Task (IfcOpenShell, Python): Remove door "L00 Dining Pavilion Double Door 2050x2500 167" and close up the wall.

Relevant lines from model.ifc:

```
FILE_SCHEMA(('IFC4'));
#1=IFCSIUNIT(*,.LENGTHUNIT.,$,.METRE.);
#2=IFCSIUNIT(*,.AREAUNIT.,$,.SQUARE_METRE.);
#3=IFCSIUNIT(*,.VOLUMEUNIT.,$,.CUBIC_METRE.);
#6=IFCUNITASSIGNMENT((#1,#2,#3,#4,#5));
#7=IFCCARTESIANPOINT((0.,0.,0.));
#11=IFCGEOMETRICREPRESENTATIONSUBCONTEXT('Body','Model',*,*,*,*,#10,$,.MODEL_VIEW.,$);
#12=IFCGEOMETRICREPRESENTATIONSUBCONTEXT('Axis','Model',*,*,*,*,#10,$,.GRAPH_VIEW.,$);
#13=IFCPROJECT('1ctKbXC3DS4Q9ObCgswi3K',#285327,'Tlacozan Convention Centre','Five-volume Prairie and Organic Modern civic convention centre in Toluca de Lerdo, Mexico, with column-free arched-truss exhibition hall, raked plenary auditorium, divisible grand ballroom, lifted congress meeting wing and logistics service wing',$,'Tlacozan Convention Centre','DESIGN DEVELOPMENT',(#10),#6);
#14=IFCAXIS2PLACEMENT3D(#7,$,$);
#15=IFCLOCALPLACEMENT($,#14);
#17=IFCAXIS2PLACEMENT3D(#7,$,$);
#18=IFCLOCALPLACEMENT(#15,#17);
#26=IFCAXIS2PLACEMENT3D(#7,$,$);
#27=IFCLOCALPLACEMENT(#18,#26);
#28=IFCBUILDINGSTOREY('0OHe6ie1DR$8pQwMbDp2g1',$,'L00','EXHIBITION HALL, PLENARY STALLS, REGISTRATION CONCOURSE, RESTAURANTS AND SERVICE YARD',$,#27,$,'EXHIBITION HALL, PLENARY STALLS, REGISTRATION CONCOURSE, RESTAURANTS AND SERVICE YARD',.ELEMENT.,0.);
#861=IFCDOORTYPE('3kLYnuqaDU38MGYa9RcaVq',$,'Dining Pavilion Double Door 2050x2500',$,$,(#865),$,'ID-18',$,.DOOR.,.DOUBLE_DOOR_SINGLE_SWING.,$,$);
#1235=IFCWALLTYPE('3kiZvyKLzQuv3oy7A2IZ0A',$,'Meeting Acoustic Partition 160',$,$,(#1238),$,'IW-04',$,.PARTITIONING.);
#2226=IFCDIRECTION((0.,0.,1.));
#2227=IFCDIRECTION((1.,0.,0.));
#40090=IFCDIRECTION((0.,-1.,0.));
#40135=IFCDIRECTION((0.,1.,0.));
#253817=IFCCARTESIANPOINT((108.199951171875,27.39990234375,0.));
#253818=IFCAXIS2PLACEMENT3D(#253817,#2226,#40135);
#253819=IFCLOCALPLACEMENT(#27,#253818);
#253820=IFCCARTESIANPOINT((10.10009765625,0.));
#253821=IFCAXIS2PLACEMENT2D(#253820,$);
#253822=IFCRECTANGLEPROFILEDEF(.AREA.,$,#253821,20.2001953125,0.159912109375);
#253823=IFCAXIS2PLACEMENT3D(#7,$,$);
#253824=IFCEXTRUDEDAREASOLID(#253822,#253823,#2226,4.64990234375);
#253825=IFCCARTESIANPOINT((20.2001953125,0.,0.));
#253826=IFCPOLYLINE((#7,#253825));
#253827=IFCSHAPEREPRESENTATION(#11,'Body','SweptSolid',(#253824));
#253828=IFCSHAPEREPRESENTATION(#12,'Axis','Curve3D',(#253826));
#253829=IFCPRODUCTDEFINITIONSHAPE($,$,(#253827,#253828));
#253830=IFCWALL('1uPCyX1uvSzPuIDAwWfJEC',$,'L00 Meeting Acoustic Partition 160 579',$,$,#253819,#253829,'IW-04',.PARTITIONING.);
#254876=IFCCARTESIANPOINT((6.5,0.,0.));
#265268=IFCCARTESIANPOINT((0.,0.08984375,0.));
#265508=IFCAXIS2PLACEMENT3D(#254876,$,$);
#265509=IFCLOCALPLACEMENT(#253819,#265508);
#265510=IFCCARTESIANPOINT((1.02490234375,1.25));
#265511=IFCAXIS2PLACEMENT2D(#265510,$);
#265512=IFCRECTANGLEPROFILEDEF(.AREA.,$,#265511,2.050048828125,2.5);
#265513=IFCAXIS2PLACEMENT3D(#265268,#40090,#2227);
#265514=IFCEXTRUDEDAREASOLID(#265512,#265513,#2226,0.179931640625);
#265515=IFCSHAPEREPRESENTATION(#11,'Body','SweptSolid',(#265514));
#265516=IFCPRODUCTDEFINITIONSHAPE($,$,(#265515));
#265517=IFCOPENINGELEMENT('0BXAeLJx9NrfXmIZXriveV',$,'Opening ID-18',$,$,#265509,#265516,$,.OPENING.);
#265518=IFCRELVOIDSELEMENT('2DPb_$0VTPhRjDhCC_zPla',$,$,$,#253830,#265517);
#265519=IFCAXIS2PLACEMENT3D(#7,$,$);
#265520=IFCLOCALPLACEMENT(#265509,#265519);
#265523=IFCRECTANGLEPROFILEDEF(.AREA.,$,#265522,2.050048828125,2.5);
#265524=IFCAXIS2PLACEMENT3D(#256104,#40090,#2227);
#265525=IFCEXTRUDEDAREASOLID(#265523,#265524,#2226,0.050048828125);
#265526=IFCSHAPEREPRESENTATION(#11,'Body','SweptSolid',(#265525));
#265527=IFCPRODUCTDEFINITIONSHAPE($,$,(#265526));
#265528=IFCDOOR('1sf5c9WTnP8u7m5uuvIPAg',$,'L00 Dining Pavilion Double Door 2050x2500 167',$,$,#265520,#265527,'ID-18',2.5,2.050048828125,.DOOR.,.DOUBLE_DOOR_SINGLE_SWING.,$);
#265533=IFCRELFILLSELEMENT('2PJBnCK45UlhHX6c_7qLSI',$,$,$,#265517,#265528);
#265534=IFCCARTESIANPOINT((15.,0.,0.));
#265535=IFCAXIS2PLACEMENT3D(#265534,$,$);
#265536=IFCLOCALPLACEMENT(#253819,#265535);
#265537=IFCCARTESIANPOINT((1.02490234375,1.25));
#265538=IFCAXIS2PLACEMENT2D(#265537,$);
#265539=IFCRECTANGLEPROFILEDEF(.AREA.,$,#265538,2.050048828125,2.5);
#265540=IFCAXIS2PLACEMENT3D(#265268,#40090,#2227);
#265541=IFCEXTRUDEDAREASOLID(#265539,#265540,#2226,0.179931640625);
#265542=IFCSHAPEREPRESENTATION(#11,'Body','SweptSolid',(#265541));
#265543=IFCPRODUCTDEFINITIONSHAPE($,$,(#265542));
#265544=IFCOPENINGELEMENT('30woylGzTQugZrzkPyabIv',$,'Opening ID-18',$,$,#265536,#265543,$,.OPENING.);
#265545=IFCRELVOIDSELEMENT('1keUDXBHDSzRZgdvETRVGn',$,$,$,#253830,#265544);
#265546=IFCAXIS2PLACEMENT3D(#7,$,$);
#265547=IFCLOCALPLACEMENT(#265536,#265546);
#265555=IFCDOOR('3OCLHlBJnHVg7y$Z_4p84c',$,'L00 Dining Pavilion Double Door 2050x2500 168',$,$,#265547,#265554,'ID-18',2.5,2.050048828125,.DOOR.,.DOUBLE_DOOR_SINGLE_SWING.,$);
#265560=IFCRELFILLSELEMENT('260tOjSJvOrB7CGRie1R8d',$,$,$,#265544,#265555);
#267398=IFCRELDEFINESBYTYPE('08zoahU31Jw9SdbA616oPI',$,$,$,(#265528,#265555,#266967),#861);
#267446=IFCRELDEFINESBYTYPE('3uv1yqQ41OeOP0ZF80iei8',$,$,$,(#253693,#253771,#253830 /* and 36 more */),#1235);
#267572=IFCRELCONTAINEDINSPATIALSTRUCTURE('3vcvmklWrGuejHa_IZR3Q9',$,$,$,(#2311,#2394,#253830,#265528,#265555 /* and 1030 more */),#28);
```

```python
import ifcopenshell
import ifcopenshell.api.feature
import ifcopenshell.api.root
import ifcopenshell.geom
import ifcopenshell.util.shape

model = ifcopenshell.open("model.ifc")
settings = ifcopenshell.geom.settings()


def volume(element):
    """Net volume in cubic metres, openings subtracted."""
    shape = ifcopenshell.geom.create_shape(settings, element)
    return ifcopenshell.util.shape.get_volume(shape.geometry)


door = model.by_guid("1sf5c9WTnP8u7m5uuvIPAg")
opening = door.FillsVoids[0].RelatingOpeningElement
wall = opening.VoidsElements[0].RelatingBuildingElement
before = volume(wall)

ifcopenshell.api.root.remove_product(model, product=door)
ifcopenshell.api.feature.remove_feature(model, feature=opening)

after = volume(wall)

print(f"wall volume {before:.3f} -> {after:.3f} m3")

model.write("model_edited.ifc")
```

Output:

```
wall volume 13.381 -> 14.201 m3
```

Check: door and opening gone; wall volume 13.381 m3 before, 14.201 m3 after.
